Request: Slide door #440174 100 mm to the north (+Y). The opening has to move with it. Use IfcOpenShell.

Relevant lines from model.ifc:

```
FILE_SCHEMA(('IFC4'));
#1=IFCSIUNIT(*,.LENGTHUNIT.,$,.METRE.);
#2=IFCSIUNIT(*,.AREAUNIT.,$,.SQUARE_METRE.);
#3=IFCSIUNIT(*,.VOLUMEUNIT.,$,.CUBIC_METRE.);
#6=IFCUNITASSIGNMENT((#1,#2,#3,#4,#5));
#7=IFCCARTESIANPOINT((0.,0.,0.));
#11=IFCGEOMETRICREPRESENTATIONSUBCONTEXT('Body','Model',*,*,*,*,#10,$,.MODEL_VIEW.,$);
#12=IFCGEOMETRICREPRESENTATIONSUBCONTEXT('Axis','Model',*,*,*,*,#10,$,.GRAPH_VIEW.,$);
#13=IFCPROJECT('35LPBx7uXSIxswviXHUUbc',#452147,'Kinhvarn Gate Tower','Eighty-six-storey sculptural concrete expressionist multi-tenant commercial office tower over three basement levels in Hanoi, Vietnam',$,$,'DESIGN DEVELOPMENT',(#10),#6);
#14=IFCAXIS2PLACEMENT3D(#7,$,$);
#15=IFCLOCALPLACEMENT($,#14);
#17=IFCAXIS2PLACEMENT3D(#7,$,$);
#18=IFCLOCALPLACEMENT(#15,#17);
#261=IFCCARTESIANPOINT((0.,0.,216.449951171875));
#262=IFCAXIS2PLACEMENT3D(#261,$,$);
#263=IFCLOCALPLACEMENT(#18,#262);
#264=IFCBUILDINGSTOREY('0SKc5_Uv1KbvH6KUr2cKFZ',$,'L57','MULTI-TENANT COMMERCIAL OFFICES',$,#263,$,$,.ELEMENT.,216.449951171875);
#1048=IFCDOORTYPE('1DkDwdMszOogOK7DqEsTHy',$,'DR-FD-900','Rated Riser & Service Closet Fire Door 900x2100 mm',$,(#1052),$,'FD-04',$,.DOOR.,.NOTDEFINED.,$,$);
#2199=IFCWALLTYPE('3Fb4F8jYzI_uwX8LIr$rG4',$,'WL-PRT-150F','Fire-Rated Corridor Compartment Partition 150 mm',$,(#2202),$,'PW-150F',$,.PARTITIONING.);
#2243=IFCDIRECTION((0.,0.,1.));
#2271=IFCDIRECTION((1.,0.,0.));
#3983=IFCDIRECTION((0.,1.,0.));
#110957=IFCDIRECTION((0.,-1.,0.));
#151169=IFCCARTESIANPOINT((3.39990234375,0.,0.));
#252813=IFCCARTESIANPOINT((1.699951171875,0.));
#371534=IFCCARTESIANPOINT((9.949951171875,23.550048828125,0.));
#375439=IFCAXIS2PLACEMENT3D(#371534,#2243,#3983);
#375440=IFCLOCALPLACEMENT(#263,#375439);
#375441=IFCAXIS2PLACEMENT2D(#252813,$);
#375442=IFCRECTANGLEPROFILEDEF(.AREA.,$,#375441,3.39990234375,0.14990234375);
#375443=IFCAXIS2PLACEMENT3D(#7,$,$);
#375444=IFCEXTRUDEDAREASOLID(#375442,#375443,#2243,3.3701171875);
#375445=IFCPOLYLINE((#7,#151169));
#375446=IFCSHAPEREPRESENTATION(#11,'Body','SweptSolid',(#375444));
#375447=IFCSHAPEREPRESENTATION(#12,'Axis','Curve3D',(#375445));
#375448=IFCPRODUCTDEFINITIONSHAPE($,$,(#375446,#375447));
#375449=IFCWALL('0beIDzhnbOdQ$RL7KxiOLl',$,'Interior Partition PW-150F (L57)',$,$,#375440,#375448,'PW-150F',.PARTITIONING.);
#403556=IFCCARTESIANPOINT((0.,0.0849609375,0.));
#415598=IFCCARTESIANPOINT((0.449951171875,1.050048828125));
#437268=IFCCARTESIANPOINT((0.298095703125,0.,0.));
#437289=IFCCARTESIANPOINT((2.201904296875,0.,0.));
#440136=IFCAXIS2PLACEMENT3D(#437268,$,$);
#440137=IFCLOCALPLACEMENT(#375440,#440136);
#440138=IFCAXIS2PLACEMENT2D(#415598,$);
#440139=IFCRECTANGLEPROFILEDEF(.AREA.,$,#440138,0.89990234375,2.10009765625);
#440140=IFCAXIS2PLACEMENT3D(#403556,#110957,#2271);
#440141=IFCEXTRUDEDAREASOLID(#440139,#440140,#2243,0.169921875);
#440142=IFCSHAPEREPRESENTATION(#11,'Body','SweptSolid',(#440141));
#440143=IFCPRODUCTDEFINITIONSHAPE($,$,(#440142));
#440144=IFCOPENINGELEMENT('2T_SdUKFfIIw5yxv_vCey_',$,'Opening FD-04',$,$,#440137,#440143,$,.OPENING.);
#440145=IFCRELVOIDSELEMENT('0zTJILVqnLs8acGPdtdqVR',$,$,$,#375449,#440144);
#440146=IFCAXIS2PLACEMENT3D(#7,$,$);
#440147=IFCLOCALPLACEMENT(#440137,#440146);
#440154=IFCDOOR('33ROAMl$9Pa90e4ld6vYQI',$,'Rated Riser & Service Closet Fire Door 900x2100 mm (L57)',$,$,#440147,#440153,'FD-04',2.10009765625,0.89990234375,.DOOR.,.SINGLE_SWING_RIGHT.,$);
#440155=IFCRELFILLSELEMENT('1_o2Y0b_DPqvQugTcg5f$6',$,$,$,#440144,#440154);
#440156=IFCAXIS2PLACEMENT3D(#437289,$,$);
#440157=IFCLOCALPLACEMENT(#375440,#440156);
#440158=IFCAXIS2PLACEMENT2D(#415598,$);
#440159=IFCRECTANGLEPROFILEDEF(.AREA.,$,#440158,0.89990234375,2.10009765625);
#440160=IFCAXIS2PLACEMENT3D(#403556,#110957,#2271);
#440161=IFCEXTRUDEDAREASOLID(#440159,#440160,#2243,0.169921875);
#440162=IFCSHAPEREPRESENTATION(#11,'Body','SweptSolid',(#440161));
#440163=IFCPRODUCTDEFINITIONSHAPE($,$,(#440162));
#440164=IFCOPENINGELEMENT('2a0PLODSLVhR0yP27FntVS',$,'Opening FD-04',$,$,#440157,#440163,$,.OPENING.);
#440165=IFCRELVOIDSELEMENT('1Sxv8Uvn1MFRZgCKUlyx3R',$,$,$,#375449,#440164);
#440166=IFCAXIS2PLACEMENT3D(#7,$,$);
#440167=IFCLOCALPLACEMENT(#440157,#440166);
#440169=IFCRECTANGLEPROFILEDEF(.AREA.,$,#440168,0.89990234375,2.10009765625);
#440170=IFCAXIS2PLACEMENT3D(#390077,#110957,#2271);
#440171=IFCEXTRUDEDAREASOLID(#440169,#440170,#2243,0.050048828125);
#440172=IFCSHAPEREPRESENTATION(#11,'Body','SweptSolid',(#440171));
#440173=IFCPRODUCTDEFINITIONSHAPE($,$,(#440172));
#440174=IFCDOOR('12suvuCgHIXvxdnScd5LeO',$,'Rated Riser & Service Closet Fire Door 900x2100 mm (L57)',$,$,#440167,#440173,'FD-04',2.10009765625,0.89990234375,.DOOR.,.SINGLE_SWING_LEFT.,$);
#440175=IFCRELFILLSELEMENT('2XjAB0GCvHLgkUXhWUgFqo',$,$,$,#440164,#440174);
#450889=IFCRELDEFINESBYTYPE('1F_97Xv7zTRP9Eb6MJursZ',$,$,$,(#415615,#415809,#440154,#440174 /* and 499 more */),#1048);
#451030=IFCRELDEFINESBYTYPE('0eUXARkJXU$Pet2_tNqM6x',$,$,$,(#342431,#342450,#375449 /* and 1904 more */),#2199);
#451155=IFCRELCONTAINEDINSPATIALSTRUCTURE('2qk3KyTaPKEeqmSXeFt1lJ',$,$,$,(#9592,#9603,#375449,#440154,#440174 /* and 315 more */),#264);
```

```python
import ifcopenshell
import ifcopenshell.api.geometry
import ifcopenshell.util.placement
import ifcopenshell.util.unit

model = ifcopenshell.open("model.ifc")
unit_scale = ifcopenshell.util.unit.calculate_unit_scale(model)

door = model.by_guid("12suvuCgHIXvxdnScd5LeO")
opening = door.FillsVoids[0].RelatingOpeningElement
wall = opening.VoidsElements[0].RelatingBuildingElement

wall_matrix = ifcopenshell.util.placement.get_local_placement(wall.ObjectPlacement)
shift = wall_matrix[:3, 0] * 0.1 / unit_scale
before = ifcopenshell.util.placement.get_local_placement(door.ObjectPlacement)[:3, 3].copy()

# The door is placed relative to its opening, so it follows when the opening moves.
matrix = ifcopenshell.util.placement.get_local_placement(opening.ObjectPlacement)
matrix[:3, 3] += shift
ifcopenshell.api.geometry.edit_object_placement(
    model, product=opening, matrix=matrix, is_si=False, should_transform_children=True
)

after = ifcopenshell.util.placement.get_local_placement(door.ObjectPlacement)[:3, 3]
print("door moved by", (after - before).round(3) + 0.0)

model.write("model_updated.ifc")
```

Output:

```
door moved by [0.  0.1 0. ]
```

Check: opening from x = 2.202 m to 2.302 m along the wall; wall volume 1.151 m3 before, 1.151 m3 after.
